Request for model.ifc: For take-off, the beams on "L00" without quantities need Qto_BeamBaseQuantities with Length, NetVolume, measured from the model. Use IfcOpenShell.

First a look at what the model holds.

```python
import ifcopenshell
import ifcopenshell.util.element
import ifcopenshell.util.unit

model = ifcopenshell.open("model.ifc")
print(model.schema)
for unit_type in ("LENGTHUNIT", "AREAUNIT", "VOLUMEUNIT"):
    print(unit_type, ifcopenshell.util.unit.calculate_unit_scale(model, unit_type))
storey = next(s for s in model.by_type("IfcBuildingStorey") if s.Name == "L00")
beams = [e for e in ifcopenshell.util.element.get_decomposition(storey) if e.is_a("IfcBeam")]
for e in sorted(beams, key=lambda e: e.id()):
    print(e.id(), e.is_a(), e.Name, list(ifcopenshell.util.element.get_psets(e, qtos_only=True)), sep=" | ")
```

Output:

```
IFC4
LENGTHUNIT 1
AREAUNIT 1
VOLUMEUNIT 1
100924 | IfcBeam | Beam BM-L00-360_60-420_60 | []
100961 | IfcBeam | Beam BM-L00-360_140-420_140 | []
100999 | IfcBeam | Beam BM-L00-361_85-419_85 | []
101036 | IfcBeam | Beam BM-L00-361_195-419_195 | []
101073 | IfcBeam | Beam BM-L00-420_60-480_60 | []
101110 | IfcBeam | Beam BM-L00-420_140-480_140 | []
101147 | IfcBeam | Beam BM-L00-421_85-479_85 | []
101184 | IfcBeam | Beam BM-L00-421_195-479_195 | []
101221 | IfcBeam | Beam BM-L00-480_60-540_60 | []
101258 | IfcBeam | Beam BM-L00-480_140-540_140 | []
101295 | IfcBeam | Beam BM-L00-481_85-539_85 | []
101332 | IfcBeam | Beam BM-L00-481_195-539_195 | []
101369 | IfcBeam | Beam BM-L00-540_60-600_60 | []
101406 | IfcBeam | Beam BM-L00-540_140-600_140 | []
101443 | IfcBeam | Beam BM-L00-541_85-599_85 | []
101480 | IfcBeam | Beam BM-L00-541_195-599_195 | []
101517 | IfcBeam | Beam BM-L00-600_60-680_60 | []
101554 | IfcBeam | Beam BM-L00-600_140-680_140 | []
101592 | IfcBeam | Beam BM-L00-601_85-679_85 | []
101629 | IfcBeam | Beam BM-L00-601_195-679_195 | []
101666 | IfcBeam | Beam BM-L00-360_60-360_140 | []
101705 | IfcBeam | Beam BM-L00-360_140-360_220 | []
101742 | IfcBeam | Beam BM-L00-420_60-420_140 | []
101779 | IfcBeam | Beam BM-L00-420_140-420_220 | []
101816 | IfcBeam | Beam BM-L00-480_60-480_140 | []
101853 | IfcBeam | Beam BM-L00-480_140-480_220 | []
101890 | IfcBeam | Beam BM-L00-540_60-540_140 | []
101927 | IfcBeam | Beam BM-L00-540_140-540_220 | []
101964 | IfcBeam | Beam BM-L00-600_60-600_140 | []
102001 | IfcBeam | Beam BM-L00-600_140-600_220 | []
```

```python
import ifcopenshell
import ifcopenshell.api.pset
import ifcopenshell.geom
import ifcopenshell.util.element
import ifcopenshell.util.shape
import ifcopenshell.util.unit

model = ifcopenshell.open("model.ifc")
unit_scale = ifcopenshell.util.unit.calculate_unit_scale(model)
volume_scale = ifcopenshell.util.unit.calculate_unit_scale(model, "VOLUMEUNIT")
settings = ifcopenshell.geom.settings()

storey = next(s for s in model.by_type("IfcBuildingStorey") if s.Name == "L00")
beams = [e for e in ifcopenshell.util.element.get_decomposition(storey) if e.is_a("IfcBeam")]

for e in sorted(beams, key=lambda e: e.id()):
    if ifcopenshell.util.element.get_psets(e, qtos_only=True, should_inherit=False):
        continue
    # Geometry comes back in metres, in the element's own axes.
    shape = ifcopenshell.geom.create_shape(settings, e)
    values = {
        "Length": ifcopenshell.util.shape.get_max_xyz(shape.geometry) / unit_scale,
        "NetVolume": ifcopenshell.util.shape.get_volume(shape.geometry) / volume_scale,
    }
    qto = ifcopenshell.api.pset.add_qto(model, product=e, name="Qto_BeamBaseQuantities")
    ifcopenshell.api.pset.edit_qto(model, qto=qto, properties=values)
    print(e.id(), {k: round(v, 3) for k, v in values.items()})

model.write("model_v2.ifc")
```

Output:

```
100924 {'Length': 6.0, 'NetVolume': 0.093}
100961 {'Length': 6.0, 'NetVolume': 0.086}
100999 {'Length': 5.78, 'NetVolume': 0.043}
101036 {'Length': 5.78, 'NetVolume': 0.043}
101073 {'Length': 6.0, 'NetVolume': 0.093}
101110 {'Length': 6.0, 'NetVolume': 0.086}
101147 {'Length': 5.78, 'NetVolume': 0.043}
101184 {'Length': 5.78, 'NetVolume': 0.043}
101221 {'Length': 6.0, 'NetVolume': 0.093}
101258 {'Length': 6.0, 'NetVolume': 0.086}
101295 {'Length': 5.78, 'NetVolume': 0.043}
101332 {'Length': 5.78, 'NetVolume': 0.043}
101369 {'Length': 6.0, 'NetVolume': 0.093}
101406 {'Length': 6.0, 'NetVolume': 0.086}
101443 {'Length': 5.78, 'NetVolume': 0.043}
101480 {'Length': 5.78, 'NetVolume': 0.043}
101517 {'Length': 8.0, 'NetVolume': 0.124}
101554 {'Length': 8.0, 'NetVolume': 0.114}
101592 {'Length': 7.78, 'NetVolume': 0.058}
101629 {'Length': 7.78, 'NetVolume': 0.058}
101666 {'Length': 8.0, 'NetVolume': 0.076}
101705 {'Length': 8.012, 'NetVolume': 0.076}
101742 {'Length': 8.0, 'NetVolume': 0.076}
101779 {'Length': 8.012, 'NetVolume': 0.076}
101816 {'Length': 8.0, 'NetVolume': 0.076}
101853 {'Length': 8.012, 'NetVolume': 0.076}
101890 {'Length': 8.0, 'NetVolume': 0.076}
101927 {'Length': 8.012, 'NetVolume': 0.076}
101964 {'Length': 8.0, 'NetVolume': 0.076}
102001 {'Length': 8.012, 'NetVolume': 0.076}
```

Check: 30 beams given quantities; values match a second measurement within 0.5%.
